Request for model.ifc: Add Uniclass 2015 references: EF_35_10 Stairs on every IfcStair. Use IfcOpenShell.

First a look at what the model holds.

```python
import ifcopenshell

model = ifcopenshell.open("model.ifc")
print(model.schema)
print("classifications:", [c.Name for c in model.by_type("IfcClassification")])
for ifc_class in ("IfcDoor", "IfcRoof", "IfcStair", "IfcWall", "IfcWindow"):
    print(ifc_class, len(model.by_type(ifc_class)))
```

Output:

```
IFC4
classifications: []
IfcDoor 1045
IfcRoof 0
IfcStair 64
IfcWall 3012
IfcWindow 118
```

```python
import ifcopenshell
import ifcopenshell.api.classification

model = ifcopenshell.open("model.ifc")

system = ifcopenshell.api.classification.add_classification(model, classification="Uniclass 2015")

codes = {
    "IfcStair": ("EF_35_10", "Stairs"),
}
for ifc_class, (code, name) in codes.items():
    products = model.by_type(ifc_class)
    ifcopenshell.api.classification.add_reference(
        model, products=products, classification=system, identification=code, name=name
    )
    print(code, len(products))

model.write("model_v2.ifc")
```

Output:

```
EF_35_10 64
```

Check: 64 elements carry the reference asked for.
